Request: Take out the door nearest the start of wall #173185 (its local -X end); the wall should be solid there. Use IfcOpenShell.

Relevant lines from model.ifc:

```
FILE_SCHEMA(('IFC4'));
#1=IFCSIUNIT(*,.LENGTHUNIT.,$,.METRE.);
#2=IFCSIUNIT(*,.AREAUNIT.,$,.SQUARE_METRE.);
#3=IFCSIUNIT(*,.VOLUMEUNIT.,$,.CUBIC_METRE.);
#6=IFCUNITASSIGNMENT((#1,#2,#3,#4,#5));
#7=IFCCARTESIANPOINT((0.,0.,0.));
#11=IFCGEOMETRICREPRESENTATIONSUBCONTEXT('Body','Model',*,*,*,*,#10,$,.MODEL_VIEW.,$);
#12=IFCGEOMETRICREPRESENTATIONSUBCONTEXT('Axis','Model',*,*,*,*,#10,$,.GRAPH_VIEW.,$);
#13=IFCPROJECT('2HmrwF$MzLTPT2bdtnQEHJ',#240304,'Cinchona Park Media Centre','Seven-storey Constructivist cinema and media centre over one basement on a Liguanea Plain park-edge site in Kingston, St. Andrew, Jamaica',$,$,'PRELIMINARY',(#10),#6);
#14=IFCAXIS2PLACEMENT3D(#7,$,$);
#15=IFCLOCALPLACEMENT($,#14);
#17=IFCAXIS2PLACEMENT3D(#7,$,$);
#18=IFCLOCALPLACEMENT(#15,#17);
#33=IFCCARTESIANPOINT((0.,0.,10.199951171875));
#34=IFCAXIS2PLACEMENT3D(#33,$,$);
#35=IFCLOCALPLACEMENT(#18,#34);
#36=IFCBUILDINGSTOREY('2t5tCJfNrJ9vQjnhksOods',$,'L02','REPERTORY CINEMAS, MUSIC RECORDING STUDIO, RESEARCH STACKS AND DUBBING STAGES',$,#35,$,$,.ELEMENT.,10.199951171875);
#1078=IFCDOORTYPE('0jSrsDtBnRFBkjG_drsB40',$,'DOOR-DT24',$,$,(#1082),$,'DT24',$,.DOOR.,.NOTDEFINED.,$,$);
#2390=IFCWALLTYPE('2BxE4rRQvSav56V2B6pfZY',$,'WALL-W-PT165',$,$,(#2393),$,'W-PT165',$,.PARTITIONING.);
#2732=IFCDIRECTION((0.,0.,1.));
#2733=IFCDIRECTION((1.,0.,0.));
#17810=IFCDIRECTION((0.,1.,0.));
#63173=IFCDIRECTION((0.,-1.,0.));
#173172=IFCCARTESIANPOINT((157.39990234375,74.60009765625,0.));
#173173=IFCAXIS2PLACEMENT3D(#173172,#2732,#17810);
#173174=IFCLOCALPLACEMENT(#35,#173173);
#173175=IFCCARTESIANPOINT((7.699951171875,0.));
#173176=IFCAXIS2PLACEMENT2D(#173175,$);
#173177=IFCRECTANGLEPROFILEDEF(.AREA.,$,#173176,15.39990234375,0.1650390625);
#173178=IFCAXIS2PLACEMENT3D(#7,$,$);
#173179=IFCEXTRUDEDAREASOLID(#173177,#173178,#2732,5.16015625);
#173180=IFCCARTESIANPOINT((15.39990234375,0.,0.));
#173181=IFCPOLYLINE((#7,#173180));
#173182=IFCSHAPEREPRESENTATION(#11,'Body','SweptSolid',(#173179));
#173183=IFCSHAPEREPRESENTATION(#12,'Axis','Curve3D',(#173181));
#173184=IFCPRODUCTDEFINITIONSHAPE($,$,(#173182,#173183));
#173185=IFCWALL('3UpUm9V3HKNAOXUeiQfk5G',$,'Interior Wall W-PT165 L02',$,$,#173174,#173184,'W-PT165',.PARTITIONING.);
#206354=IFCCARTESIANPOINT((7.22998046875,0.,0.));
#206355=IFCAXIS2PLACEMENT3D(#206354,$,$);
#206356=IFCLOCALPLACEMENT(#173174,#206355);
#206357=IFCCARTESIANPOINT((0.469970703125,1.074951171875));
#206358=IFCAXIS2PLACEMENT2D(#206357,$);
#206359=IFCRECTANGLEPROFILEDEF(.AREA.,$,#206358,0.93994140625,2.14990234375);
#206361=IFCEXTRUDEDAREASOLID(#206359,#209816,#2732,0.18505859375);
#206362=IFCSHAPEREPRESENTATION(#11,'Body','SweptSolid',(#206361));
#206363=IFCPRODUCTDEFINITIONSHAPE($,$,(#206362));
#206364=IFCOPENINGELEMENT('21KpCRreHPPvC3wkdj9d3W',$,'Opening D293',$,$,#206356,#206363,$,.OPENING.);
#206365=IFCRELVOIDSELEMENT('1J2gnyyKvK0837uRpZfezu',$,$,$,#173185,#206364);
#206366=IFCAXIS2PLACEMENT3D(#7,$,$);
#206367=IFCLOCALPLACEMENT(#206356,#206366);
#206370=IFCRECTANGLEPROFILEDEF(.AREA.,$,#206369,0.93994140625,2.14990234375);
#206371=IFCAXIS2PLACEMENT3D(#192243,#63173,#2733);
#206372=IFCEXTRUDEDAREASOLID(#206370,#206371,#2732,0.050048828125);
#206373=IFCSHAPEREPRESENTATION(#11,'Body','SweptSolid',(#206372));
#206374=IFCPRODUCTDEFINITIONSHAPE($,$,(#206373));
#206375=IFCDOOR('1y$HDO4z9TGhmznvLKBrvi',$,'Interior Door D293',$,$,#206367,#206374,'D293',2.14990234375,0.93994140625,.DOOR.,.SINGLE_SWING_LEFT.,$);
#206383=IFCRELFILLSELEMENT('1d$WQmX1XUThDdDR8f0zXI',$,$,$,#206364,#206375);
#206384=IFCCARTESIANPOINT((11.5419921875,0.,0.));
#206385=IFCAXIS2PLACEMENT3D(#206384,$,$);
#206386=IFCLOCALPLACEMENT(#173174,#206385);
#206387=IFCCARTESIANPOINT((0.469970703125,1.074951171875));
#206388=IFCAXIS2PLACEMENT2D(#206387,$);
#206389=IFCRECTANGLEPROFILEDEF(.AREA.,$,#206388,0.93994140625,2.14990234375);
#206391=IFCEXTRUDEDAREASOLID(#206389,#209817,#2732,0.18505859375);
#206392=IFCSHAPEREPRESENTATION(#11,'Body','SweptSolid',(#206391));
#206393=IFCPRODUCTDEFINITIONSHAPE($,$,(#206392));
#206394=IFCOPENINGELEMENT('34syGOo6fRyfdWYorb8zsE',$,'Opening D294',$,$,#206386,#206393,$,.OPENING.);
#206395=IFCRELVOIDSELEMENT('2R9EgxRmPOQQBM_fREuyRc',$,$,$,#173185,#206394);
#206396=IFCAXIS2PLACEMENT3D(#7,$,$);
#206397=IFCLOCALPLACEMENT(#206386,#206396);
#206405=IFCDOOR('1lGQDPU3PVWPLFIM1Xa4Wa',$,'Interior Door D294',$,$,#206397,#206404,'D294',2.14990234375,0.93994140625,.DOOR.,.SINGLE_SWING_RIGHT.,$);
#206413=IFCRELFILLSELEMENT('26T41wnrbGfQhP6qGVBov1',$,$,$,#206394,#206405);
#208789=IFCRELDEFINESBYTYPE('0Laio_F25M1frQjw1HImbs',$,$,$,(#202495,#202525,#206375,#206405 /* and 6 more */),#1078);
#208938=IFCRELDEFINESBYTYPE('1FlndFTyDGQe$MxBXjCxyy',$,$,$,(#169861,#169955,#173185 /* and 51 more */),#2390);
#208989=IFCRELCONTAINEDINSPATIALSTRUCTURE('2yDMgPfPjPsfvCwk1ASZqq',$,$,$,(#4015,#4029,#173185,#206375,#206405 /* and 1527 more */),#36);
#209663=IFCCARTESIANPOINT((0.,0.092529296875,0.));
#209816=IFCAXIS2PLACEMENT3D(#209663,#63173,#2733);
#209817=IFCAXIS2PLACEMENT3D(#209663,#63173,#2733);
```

```python
import ifcopenshell
import ifcopenshell.api.feature
import ifcopenshell.api.root
import ifcopenshell.geom
import ifcopenshell.util.shape

model = ifcopenshell.open("model.ifc")
settings = ifcopenshell.geom.settings()


def volume(element):
    """Net volume in cubic metres, openings subtracted."""
    shape = ifcopenshell.geom.create_shape(settings, element)
    return ifcopenshell.util.shape.get_volume(shape.geometry)


door = model.by_id(206375)
opening = door.FillsVoids[0].RelatingOpeningElement
wall = opening.VoidsElements[0].RelatingBuildingElement
before = volume(wall)

ifcopenshell.api.root.remove_product(model, product=door)
ifcopenshell.api.feature.remove_feature(model, feature=opening)

after = volume(wall)

print(f"wall volume {before:.3f} -> {after:.3f} m3")

model.write("model_updated.ifc")
```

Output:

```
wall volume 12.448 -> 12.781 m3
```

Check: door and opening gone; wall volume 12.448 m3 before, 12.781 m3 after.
